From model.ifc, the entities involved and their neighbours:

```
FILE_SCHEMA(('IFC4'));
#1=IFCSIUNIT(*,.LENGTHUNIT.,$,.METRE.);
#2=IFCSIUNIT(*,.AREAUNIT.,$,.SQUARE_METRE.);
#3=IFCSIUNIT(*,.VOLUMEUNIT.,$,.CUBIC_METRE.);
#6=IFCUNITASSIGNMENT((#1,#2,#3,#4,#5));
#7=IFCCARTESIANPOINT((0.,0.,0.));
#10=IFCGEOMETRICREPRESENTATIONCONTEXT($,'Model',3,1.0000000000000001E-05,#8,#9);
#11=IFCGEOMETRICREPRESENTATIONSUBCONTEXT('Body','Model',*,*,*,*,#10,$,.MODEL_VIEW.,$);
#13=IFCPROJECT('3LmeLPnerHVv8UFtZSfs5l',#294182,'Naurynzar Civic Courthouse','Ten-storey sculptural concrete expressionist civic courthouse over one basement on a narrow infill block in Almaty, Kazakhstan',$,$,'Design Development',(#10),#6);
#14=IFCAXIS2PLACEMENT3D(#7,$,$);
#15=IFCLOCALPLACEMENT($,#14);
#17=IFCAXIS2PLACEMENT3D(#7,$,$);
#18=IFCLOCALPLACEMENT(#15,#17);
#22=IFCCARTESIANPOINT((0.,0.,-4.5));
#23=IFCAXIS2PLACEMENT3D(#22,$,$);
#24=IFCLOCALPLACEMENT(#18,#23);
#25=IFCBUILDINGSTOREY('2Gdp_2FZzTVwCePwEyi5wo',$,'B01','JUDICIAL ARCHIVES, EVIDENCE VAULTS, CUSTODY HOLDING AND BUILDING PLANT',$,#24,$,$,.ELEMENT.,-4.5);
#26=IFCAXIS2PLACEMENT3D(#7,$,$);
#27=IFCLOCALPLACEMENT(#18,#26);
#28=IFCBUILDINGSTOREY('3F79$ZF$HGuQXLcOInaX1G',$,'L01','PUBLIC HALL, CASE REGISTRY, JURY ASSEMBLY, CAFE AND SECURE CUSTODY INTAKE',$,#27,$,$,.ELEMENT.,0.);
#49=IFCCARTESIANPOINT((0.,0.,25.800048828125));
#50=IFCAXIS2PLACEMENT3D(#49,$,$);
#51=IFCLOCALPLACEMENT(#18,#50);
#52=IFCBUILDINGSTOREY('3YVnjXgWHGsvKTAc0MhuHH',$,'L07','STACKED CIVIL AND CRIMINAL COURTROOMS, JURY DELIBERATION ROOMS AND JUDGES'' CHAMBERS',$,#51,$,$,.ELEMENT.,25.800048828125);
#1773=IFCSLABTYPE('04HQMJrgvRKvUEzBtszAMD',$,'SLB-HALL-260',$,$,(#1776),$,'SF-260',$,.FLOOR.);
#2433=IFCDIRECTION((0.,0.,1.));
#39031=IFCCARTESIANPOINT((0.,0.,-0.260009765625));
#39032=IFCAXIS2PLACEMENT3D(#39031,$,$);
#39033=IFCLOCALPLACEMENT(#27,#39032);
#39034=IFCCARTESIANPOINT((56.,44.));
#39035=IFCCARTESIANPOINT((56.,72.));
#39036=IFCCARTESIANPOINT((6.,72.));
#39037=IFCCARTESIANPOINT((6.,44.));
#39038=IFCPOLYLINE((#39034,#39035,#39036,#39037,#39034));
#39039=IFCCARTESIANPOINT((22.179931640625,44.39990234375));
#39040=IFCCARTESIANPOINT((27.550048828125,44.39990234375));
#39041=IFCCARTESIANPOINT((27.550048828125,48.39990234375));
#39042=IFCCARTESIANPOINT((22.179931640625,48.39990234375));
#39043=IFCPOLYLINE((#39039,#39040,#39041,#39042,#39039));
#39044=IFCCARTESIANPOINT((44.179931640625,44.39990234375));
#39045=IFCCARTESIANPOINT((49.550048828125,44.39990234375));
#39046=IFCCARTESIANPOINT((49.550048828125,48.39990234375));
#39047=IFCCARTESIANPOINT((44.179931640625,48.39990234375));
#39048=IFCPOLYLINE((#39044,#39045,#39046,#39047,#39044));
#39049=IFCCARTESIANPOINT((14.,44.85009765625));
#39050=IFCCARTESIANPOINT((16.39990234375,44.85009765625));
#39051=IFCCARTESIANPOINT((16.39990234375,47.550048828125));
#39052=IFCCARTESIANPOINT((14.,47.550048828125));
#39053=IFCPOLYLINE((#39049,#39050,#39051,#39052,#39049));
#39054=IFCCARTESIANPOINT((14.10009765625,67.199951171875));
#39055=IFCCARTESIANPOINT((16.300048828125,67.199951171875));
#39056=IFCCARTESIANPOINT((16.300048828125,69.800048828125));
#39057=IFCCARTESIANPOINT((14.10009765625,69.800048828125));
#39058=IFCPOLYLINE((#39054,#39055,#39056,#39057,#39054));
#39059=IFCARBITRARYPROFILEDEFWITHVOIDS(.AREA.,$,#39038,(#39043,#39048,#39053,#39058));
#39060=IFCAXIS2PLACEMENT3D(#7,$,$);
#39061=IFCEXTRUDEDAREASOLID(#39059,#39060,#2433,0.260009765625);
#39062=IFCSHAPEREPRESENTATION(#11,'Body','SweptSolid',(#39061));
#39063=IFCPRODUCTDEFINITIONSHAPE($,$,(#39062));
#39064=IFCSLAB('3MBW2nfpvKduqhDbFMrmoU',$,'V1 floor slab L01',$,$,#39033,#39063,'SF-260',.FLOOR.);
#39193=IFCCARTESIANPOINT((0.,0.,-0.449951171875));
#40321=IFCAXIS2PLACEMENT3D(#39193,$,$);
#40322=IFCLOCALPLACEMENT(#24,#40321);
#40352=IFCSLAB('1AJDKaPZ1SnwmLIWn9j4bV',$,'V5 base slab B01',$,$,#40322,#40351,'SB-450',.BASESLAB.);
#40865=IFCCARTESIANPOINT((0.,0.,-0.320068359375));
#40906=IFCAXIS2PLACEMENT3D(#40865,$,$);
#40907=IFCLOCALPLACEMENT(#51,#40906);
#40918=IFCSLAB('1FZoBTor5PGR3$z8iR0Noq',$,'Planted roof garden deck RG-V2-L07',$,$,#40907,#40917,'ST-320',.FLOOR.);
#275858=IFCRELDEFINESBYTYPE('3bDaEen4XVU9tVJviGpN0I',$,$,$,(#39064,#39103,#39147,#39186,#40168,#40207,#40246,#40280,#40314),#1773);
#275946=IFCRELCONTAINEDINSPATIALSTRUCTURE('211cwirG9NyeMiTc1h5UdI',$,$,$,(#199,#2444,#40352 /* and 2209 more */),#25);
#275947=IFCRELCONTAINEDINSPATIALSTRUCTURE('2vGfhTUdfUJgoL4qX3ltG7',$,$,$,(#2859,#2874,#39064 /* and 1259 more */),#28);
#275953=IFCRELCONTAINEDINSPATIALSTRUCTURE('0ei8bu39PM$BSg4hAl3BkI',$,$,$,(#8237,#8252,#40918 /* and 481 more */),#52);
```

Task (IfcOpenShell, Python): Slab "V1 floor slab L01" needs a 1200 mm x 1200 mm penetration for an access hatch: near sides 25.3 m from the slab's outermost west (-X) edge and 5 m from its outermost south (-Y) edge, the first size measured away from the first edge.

```python
import numpy as np
import ifcopenshell
import ifcopenshell.api.feature
import ifcopenshell.api.geometry
import ifcopenshell.api.root
import ifcopenshell.geom
import ifcopenshell.util.placement
import ifcopenshell.util.representation
import ifcopenshell.util.shape
import ifcopenshell.util.unit

model = ifcopenshell.open("model.ifc")
unit_scale = ifcopenshell.util.unit.calculate_unit_scale(model)
settings = ifcopenshell.geom.settings()


def volume(element):
    """Net volume in cubic metres, openings subtracted."""
    shape = ifcopenshell.geom.create_shape(settings, element)
    return ifcopenshell.util.shape.get_volume(shape.geometry)


slab = model.by_guid("3MBW2nfpvKduqhDbFMrmoU")
before = volume(slab)

# Extent in the slab's own axes, in metres. The edges named are its -X and -Y sides.
slab_shape = ifcopenshell.geom.create_shape(settings, slab)
vertices = ifcopenshell.util.shape.get_vertices(slab_shape.geometry)
x_min, y_min, bottom = vertices.min(axis=0)
top = vertices[:, 2].max()

opening = ifcopenshell.api.root.create_entity(model, ifc_class="IfcOpeningElement", name="Access hatch opening", predefined_type="OPENING")
context = ifcopenshell.util.representation.get_context(model, "Model", "Body", "MODEL_VIEW")
width, depth = 1.2, 1.2
outline = [(0.0, 0.0), (width, 0.0), (width, depth), (0.0, depth), (0.0, 0.0)]
# Overshoot both faces by 50 mm so the cut is clean.
shape = ifcopenshell.api.geometry.add_slab_representation(
    model, context=context, depth=top - bottom + 0.1, polyline=outline
)
ifcopenshell.api.geometry.assign_representation(model, product=opening, representation=shape)

matrix = ifcopenshell.util.placement.get_local_placement(slab.ObjectPlacement)
matrix[:, 3] = matrix @ np.append(np.array([x_min + 25.3, y_min + 5, bottom - 0.05]) / unit_scale, 1.0)
ifcopenshell.api.geometry.edit_object_placement(model, product=opening, matrix=matrix, is_si=False)
ifcopenshell.api.feature.add_feature(model, feature=opening, element=slab)

after = volume(slab)

print(f"slab volume {before:.3f} -> {after:.3f} m3")

model.write("model_updated.ifc")
```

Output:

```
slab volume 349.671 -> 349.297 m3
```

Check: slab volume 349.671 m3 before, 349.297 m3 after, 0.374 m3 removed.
